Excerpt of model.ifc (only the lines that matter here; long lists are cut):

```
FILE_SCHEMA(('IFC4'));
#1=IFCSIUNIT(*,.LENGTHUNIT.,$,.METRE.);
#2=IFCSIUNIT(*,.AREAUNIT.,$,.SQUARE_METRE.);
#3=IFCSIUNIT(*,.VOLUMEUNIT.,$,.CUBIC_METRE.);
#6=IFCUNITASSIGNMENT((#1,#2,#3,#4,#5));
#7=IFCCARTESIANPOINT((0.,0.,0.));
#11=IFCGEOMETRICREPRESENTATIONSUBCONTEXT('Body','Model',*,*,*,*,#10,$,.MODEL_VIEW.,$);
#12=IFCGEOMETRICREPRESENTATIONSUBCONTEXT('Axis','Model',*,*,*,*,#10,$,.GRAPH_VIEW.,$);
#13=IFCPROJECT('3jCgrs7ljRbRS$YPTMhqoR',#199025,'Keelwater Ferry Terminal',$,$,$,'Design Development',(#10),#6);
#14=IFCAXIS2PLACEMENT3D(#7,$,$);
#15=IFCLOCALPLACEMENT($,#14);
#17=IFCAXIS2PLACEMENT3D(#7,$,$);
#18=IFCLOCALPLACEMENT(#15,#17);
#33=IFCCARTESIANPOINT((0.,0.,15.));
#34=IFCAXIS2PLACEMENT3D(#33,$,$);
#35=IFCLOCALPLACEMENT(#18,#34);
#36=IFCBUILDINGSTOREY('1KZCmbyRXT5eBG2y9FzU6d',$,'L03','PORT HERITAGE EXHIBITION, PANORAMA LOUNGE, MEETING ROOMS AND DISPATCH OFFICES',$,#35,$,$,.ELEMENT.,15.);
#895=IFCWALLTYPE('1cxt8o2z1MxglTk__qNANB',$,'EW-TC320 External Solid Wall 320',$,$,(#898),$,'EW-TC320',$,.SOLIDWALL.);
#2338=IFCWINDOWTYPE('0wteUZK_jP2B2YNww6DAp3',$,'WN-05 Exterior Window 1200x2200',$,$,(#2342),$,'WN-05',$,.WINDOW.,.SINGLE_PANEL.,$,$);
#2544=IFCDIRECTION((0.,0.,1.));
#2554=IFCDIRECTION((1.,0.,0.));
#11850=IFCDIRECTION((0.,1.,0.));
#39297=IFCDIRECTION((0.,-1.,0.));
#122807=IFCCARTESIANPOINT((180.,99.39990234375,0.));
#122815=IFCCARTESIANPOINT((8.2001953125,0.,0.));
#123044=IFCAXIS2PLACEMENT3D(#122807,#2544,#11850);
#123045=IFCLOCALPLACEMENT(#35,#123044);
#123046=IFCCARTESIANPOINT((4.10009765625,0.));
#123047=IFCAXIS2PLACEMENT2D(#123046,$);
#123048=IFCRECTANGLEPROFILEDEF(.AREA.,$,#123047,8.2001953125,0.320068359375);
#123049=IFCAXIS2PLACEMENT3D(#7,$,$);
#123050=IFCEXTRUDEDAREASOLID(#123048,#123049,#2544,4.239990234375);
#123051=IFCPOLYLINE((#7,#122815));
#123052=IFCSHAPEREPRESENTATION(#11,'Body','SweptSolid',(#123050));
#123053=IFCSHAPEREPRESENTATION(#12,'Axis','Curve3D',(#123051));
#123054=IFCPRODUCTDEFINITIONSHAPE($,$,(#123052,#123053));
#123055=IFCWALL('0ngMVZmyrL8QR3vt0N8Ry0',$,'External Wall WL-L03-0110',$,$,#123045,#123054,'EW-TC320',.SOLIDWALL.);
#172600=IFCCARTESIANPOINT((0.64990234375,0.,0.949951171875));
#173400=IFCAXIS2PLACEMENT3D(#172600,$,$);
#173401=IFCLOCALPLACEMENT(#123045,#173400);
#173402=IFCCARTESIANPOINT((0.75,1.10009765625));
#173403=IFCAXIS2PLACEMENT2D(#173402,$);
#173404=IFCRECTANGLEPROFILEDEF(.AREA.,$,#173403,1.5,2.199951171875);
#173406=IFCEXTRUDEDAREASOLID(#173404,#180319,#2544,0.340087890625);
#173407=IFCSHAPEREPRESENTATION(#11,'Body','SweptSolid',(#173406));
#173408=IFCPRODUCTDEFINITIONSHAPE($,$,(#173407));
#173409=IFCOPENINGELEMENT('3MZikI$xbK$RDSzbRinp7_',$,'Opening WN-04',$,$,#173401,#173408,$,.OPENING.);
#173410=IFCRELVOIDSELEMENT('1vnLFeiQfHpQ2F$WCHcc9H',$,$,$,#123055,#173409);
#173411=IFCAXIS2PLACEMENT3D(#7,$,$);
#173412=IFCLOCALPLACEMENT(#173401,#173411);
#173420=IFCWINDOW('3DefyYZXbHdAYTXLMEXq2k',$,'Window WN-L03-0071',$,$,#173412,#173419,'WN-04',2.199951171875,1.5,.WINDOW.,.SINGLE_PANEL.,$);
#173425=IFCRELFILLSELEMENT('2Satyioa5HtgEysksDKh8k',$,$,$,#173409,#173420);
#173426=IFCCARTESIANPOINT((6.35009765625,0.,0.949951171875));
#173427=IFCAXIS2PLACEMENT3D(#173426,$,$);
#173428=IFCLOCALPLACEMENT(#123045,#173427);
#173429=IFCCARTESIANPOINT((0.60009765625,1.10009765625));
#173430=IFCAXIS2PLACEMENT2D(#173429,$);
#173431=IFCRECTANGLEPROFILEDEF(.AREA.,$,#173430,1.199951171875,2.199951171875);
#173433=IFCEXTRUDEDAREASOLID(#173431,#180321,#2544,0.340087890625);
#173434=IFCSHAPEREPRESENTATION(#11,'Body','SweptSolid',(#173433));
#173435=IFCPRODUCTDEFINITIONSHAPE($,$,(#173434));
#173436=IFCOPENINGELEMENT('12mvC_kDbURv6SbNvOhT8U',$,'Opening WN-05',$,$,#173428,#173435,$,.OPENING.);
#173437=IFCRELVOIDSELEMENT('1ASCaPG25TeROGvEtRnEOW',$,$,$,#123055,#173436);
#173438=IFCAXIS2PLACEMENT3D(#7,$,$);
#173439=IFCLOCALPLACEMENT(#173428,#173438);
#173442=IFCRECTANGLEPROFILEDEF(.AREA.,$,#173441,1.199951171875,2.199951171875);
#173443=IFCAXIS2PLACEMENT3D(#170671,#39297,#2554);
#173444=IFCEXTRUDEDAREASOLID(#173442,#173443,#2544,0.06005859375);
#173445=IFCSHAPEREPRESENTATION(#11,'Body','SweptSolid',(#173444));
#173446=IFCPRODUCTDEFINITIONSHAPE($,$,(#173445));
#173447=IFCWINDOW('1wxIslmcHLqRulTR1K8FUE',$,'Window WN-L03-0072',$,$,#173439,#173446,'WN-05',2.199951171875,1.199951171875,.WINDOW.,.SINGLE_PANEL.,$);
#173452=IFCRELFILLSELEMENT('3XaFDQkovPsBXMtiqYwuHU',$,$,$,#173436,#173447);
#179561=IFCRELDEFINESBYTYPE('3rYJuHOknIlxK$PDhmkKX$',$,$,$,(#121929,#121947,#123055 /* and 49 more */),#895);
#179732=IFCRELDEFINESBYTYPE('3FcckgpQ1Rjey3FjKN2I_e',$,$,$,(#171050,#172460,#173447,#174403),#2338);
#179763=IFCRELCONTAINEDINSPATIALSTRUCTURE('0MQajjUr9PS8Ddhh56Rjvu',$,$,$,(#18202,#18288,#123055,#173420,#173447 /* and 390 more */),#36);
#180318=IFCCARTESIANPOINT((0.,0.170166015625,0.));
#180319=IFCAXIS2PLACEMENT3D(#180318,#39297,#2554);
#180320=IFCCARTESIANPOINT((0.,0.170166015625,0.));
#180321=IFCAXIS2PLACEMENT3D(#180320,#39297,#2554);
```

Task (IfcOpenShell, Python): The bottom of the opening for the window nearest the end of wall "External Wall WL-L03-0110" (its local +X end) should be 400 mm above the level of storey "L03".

```python
import numpy as np
import ifcopenshell
import ifcopenshell.api.geometry
import ifcopenshell.geom
import ifcopenshell.util.element
import ifcopenshell.util.placement
import ifcopenshell.util.shape
import ifcopenshell.util.unit

model = ifcopenshell.open("model.ifc")
unit_scale = ifcopenshell.util.unit.calculate_unit_scale(model)

window = model.by_guid("1wxIslmcHLqRulTR1K8FUE")
opening = window.FillsVoids[0].RelatingOpeningElement
storey = ifcopenshell.util.element.get_container(window, ifc_class="IfcBuildingStorey")
level = ifcopenshell.util.placement.get_local_placement(storey.ObjectPlacement)[2, 3]

# The opening's origin need not be at the sill, so measure its lowest point.
shape = ifcopenshell.geom.create_shape(ifcopenshell.geom.settings(), opening)
bottom = ifcopenshell.util.shape.get_shape_bottom_elevation(shape, shape.geometry) / unit_scale
dz = level + 0.4 / unit_scale - bottom

shift = np.array([0.0, 0.0, dz])
# The window is placed relative to its opening, so it follows when the opening moves.
matrix = ifcopenshell.util.placement.get_local_placement(opening.ObjectPlacement)
matrix[:3, 3] += shift
ifcopenshell.api.geometry.edit_object_placement(
    model, product=opening, matrix=matrix, is_si=False, should_transform_children=True
)

print(f"moved by {dz * unit_scale:+.3f} m")

model.write("model_edited.ifc")
```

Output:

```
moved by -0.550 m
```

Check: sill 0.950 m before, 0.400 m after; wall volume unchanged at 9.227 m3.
